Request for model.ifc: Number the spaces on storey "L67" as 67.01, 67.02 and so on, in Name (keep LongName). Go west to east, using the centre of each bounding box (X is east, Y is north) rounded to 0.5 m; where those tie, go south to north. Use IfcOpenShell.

First a look at what the model holds.

```python
import ifcopenshell
import ifcopenshell.util.element
import ifcopenshell.util.placement

model = ifcopenshell.open("model.ifc")
print(model.schema)
storey = next(s for s in model.by_type("IfcBuildingStorey") if s.Name == "L67")
spaces = [e for e in ifcopenshell.util.element.get_decomposition(storey) if e.is_a("IfcSpace")]
for e in sorted(spaces, key=lambda e: e.id()):
    origin = ifcopenshell.util.placement.get_local_placement(e.ObjectPlacement)[:3, 3]
    print(e.id(), e.Name, e.LongName, origin.round(2) + 0.0, sep=" | ")
```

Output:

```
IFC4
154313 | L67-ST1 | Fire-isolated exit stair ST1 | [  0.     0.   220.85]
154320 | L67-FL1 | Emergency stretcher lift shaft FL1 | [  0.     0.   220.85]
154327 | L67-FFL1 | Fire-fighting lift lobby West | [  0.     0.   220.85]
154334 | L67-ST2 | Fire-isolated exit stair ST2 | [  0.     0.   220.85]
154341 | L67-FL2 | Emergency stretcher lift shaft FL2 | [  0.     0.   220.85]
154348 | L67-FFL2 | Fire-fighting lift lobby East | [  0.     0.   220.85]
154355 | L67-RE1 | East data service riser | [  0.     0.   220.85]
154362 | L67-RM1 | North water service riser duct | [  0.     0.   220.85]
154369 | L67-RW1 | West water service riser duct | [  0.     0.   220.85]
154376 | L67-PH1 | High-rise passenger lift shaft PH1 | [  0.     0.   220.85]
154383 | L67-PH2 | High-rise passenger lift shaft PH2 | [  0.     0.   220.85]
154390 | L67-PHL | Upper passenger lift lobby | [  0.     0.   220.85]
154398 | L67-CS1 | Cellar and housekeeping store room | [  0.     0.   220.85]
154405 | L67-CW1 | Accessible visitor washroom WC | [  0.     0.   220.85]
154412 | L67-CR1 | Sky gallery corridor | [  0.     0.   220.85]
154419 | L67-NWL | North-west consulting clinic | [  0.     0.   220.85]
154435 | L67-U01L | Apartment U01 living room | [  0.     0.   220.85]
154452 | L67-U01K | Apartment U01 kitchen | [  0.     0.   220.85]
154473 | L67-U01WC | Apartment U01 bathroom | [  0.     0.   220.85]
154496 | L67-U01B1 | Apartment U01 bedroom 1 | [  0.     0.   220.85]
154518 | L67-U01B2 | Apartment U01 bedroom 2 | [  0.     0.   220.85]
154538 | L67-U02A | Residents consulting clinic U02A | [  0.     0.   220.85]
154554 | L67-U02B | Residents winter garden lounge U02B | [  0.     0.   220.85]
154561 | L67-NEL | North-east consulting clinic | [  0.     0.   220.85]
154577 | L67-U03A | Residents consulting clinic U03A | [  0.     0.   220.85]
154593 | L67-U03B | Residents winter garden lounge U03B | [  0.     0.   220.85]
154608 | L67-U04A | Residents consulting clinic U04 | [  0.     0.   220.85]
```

```python
import ifcopenshell
import ifcopenshell.geom
import ifcopenshell.util.element
import ifcopenshell.util.shape

model = ifcopenshell.open("model.ifc")
settings = ifcopenshell.geom.settings()
settings.set("use-world-coords", True)


def centre(element):
    shape = ifcopenshell.geom.create_shape(settings, element)
    return ifcopenshell.util.shape.get_bbox_centroid(shape.geometry)


storey = next(s for s in model.by_type("IfcBuildingStorey") if s.Name == "L67")
spaces = [e for e in ifcopenshell.util.element.get_decomposition(storey) if e.is_a("IfcSpace")]

# Insertion points can sit at a corner or the storey origin, so sort by the geometry (in metres).
centres = {e: centre(e) for e in spaces}
spaces.sort(key=lambda e: (round(centres[e][0] / 0.5), centres[e][1]))

for i, e in enumerate(spaces, start=1):
    number = f"67.{i:02d}"
    e.Name = number
    print(e.id(), number)

model.write("model_rev.ifc")
```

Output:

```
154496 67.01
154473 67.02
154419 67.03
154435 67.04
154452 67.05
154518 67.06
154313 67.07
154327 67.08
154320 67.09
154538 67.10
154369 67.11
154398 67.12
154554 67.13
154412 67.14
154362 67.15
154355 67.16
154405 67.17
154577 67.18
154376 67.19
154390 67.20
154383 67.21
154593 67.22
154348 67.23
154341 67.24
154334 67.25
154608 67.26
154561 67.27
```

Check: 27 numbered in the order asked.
